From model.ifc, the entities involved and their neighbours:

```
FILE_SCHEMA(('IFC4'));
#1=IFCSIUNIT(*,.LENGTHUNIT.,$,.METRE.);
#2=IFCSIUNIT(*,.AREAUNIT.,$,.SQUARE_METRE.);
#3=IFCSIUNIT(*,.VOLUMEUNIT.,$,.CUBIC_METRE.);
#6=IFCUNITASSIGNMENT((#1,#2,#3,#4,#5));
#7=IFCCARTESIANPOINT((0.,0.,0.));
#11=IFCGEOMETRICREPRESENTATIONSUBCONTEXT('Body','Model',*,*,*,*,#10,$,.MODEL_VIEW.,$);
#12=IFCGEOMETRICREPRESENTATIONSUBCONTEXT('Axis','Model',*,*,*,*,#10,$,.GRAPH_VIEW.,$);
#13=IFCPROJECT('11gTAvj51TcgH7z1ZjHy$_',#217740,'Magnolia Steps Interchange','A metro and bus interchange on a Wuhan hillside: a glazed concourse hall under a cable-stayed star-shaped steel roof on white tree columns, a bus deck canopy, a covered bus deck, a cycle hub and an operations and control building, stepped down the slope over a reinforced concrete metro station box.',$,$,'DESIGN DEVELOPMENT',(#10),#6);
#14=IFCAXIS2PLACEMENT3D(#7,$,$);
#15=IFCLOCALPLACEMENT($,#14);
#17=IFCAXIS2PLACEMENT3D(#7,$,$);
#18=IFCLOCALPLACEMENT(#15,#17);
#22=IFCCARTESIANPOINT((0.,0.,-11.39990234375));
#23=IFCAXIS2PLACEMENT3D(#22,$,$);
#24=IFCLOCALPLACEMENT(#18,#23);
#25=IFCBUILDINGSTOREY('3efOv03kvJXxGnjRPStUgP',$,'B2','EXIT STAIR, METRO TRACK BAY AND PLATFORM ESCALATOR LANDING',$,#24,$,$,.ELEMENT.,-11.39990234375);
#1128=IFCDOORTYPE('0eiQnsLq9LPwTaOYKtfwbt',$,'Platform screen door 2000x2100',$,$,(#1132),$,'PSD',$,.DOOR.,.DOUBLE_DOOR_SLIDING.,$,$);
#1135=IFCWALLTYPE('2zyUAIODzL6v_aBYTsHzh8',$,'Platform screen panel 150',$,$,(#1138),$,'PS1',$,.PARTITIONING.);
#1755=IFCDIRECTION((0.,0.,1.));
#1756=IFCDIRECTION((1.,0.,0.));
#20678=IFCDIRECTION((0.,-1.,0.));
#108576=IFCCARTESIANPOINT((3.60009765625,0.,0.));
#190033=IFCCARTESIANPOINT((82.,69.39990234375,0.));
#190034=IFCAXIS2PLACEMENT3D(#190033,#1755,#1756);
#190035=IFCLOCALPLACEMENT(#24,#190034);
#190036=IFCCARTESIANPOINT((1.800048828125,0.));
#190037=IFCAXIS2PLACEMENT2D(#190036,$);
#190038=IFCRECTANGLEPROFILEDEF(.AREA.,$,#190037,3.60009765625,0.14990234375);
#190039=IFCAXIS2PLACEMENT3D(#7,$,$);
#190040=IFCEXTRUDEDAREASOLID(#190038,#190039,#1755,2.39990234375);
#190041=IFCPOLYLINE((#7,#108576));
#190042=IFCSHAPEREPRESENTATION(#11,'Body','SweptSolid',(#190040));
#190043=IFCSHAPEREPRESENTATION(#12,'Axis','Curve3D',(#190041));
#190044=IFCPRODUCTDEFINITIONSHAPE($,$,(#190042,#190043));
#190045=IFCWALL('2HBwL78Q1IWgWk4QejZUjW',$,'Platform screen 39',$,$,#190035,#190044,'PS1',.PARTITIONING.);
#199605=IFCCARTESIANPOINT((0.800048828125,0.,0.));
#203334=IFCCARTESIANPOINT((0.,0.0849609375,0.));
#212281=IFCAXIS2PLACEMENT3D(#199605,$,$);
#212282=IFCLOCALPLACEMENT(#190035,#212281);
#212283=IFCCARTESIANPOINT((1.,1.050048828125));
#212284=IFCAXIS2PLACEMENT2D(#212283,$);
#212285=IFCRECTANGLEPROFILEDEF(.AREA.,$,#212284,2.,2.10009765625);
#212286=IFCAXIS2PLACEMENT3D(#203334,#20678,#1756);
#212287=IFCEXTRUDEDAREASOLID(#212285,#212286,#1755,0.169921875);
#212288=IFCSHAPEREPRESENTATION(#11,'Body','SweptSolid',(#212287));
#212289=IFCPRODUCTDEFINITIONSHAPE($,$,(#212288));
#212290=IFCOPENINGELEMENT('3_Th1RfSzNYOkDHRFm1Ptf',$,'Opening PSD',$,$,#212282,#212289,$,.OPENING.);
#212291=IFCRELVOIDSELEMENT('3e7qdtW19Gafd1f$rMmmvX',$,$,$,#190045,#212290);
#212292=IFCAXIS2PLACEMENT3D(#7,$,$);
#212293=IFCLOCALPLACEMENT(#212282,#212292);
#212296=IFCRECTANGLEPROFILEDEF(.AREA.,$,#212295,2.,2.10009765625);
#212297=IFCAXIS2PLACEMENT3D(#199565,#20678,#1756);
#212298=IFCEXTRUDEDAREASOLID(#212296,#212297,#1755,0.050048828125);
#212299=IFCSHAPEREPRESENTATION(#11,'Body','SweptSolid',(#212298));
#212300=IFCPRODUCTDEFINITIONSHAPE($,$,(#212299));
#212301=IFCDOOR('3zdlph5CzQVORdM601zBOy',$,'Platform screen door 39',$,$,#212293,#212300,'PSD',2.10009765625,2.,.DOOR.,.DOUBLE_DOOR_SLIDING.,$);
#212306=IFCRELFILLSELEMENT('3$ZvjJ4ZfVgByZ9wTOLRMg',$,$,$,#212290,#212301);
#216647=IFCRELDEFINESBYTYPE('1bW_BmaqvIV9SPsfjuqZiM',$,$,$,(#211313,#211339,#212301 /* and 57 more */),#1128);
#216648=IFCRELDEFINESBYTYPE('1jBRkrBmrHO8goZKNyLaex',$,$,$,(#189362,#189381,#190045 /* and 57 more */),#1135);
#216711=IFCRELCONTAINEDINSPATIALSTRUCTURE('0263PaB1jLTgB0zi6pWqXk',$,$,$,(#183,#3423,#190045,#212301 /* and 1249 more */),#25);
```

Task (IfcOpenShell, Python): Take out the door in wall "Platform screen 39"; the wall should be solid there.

```python
import ifcopenshell
import ifcopenshell.api.feature
import ifcopenshell.api.root
import ifcopenshell.geom
import ifcopenshell.util.shape

model = ifcopenshell.open("model.ifc")
settings = ifcopenshell.geom.settings()


def volume(element):
    """Net volume in cubic metres, openings subtracted."""
    shape = ifcopenshell.geom.create_shape(settings, element)
    return ifcopenshell.util.shape.get_volume(shape.geometry)


door = model.by_guid("3zdlph5CzQVORdM601zBOy")
opening = door.FillsVoids[0].RelatingOpeningElement
wall = opening.VoidsElements[0].RelatingBuildingElement
before = volume(wall)

ifcopenshell.api.root.remove_product(model, product=door)
ifcopenshell.api.feature.remove_feature(model, feature=opening)

after = volume(wall)

print(f"wall volume {before:.3f} -> {after:.3f} m3")

model.write("model_updated.ifc")
```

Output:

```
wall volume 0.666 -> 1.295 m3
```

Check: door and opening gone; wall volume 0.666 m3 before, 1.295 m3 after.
